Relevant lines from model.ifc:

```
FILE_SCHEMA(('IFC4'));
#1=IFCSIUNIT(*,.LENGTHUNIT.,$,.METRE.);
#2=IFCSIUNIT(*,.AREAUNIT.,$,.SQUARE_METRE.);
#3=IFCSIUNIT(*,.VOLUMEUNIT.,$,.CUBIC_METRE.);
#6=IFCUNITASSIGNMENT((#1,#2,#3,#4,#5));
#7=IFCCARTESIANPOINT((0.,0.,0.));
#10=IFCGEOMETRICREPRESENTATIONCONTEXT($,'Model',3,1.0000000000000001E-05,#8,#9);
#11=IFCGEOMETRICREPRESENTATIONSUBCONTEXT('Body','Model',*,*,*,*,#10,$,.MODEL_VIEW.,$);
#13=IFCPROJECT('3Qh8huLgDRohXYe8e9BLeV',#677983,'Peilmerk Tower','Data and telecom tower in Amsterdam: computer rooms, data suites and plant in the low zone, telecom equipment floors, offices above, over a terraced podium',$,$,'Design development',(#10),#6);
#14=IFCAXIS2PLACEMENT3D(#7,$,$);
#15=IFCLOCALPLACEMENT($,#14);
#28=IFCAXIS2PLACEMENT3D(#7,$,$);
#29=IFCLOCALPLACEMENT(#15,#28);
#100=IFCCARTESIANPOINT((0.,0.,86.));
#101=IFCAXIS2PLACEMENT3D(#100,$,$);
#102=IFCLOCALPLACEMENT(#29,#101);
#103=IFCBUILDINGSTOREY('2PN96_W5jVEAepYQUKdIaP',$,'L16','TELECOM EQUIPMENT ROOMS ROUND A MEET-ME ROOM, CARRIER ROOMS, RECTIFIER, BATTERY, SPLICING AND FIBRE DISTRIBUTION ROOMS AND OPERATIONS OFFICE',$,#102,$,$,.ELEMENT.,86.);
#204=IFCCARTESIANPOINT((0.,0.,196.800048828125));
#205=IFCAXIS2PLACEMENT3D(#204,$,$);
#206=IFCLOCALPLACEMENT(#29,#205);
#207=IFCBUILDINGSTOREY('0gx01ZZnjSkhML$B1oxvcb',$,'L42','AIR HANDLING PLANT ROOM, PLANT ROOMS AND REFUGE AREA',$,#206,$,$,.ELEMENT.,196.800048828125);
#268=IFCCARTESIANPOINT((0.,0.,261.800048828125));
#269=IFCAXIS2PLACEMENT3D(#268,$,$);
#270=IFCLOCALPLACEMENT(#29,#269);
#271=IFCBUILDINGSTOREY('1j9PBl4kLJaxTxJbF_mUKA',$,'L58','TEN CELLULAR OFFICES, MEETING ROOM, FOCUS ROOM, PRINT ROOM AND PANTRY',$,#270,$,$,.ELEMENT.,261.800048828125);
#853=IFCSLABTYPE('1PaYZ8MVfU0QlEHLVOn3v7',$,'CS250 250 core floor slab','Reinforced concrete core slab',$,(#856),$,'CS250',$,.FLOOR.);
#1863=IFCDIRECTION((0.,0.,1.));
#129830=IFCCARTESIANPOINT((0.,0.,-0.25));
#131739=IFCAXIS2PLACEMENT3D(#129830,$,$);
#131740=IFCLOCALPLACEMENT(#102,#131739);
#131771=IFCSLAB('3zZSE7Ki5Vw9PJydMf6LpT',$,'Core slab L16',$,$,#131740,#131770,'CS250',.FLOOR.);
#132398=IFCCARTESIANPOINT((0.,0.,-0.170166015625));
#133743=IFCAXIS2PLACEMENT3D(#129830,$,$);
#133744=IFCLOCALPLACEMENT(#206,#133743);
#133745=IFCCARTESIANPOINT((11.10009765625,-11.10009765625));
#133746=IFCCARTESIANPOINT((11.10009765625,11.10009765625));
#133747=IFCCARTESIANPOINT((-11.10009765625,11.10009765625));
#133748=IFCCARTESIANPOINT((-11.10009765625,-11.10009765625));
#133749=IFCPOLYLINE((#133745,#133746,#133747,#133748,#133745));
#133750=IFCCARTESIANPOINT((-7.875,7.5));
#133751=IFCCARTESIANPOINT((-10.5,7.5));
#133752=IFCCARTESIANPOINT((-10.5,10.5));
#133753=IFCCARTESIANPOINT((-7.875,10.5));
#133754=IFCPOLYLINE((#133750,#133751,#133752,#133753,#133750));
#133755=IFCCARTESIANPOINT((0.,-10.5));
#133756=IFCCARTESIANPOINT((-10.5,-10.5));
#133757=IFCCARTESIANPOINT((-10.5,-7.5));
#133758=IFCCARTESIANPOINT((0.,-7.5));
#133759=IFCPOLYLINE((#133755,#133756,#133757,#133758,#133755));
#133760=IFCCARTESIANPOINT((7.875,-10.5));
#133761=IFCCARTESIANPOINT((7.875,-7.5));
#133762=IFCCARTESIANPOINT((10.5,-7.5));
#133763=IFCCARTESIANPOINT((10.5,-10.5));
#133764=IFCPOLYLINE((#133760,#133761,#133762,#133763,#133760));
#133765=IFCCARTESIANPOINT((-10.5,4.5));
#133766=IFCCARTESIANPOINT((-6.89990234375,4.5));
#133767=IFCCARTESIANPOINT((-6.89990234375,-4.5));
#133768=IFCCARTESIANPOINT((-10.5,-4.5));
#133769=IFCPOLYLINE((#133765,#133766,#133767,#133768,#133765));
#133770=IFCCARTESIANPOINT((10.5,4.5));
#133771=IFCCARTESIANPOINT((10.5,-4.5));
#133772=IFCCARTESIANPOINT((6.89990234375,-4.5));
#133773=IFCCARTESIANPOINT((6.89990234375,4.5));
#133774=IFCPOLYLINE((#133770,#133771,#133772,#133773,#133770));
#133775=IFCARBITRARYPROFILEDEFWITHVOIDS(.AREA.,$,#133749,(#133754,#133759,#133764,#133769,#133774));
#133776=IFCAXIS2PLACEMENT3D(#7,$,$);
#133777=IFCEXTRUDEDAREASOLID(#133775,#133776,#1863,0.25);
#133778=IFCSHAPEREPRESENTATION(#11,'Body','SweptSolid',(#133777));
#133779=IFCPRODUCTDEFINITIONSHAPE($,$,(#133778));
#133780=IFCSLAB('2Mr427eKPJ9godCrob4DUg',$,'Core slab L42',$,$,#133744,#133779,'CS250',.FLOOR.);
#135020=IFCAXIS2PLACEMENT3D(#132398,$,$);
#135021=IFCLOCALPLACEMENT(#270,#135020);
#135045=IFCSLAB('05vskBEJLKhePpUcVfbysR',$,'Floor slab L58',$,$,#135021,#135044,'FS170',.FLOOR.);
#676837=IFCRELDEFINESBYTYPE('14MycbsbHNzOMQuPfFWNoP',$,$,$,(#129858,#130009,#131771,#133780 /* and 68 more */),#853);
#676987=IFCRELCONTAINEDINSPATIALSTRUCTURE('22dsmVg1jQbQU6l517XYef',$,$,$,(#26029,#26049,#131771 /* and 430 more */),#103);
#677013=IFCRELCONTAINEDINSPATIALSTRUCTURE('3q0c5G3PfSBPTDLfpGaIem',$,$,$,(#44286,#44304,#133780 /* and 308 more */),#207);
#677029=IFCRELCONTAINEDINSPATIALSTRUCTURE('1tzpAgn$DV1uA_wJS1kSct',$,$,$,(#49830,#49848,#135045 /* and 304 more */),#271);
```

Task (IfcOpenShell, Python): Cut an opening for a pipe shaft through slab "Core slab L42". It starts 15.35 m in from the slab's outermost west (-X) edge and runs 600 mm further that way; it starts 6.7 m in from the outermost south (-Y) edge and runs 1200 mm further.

```python
import numpy as np
import ifcopenshell
import ifcopenshell.api.feature
import ifcopenshell.api.geometry
import ifcopenshell.api.root
import ifcopenshell.geom
import ifcopenshell.util.placement
import ifcopenshell.util.representation
import ifcopenshell.util.shape
import ifcopenshell.util.unit

model = ifcopenshell.open("model.ifc")
unit_scale = ifcopenshell.util.unit.calculate_unit_scale(model)
settings = ifcopenshell.geom.settings()


def volume(element):
    """Net volume in cubic metres, openings subtracted."""
    shape = ifcopenshell.geom.create_shape(settings, element)
    return ifcopenshell.util.shape.get_volume(shape.geometry)


slab = model.by_guid("2Mr427eKPJ9godCrob4DUg")
before = volume(slab)

# Extent in the slab's own axes, in metres. The edges named are its -X and -Y sides.
slab_shape = ifcopenshell.geom.create_shape(settings, slab)
vertices = ifcopenshell.util.shape.get_vertices(slab_shape.geometry)
x_min, y_min, bottom = vertices.min(axis=0)
top = vertices[:, 2].max()

opening = ifcopenshell.api.root.create_entity(model, ifc_class="IfcOpeningElement", name="Pipe shaft opening", predefined_type="OPENING")
context = ifcopenshell.util.representation.get_context(model, "Model", "Body", "MODEL_VIEW")
width, depth = 0.6, 1.2
outline = [(0.0, 0.0), (width, 0.0), (width, depth), (0.0, depth), (0.0, 0.0)]
# Overshoot both faces by 50 mm so the cut is clean.
shape = ifcopenshell.api.geometry.add_slab_representation(
    model, context=context, depth=top - bottom + 0.1, polyline=outline
)
ifcopenshell.api.geometry.assign_representation(model, product=opening, representation=shape)

matrix = ifcopenshell.util.placement.get_local_placement(slab.ObjectPlacement)
matrix[:, 3] = matrix @ np.append(np.array([x_min + 15.35, y_min + 6.7, bottom - 0.05]) / unit_scale, 1.0)
ifcopenshell.api.geometry.edit_object_placement(model, product=opening, matrix=matrix, is_si=False)
ifcopenshell.api.feature.add_feature(model, feature=opening, element=slab)

after = volume(slab)

print(f"slab volume {before:.3f} -> {after:.3f} m3")

model.write("model_edited.ifc")
```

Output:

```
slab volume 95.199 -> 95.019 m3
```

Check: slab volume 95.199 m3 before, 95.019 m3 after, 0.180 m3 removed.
